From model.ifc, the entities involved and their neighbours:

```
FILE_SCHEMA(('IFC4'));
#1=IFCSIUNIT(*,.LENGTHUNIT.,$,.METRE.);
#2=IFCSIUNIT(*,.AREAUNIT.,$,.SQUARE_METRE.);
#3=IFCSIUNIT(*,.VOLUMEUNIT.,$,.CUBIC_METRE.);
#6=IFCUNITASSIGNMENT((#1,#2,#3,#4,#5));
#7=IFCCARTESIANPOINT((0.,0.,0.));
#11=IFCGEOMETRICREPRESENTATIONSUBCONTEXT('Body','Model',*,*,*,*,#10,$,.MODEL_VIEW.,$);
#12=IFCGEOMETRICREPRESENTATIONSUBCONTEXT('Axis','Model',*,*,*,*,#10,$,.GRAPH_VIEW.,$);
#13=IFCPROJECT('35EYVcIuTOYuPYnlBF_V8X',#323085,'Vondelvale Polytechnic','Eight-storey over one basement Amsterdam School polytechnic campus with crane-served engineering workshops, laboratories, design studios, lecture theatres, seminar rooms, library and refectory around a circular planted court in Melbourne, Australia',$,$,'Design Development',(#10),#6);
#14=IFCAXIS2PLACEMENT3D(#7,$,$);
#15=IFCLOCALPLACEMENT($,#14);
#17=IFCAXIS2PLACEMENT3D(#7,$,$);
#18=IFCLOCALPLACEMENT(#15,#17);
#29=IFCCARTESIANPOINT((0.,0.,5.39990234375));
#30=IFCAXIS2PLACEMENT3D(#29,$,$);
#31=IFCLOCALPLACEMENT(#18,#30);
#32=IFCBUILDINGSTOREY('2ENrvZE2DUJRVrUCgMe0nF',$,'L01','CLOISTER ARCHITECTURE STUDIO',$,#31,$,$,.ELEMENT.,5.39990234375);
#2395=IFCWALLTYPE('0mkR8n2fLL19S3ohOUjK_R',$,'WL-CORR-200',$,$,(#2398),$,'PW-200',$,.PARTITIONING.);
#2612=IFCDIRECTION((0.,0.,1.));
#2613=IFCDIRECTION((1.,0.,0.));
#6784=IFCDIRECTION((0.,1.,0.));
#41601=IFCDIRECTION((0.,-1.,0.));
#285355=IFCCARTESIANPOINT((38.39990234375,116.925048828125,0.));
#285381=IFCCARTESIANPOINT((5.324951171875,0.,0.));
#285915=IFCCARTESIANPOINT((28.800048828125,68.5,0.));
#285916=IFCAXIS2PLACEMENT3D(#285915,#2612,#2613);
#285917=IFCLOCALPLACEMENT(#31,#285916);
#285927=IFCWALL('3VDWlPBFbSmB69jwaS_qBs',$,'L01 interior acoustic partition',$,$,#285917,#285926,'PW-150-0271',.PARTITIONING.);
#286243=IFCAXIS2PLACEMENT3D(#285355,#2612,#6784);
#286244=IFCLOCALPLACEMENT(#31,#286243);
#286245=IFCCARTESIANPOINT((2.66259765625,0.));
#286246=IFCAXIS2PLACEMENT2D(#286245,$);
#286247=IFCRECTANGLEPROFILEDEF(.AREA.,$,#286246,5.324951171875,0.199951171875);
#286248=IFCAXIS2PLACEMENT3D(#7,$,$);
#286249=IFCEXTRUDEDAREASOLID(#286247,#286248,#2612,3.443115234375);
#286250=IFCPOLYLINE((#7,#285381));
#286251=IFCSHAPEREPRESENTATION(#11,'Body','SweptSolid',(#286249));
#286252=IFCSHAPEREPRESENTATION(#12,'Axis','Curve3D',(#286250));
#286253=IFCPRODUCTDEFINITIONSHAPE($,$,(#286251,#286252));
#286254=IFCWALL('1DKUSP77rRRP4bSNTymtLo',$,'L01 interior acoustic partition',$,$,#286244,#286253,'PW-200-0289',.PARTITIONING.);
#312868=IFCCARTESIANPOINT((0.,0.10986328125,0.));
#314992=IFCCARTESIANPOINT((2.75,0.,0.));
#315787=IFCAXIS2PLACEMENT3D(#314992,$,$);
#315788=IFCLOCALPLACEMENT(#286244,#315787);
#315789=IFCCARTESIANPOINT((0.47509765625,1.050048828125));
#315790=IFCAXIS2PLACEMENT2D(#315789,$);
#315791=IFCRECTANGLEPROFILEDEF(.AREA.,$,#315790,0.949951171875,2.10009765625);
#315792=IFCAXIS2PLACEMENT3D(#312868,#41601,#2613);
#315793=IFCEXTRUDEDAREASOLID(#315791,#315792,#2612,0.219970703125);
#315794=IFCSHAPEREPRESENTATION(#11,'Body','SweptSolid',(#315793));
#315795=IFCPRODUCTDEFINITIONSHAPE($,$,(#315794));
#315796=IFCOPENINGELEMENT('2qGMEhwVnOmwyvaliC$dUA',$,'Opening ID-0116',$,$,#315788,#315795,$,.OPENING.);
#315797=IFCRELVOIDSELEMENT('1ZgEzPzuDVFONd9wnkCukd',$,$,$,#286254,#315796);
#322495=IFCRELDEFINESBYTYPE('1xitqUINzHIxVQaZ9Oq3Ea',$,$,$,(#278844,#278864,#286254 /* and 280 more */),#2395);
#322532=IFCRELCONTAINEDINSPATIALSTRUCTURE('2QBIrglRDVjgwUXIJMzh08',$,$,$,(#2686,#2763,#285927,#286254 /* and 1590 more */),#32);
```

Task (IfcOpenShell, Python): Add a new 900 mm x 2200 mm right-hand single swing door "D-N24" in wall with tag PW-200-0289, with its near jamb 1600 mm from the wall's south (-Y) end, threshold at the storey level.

```python
import numpy as np
import ifcopenshell
import ifcopenshell.api.feature
import ifcopenshell.api.geometry
import ifcopenshell.api.root
import ifcopenshell.api.spatial
import ifcopenshell.geom
import ifcopenshell.util.element
import ifcopenshell.util.placement
import ifcopenshell.util.representation
import ifcopenshell.util.shape
import ifcopenshell.util.unit

model = ifcopenshell.open("model.ifc")
unit_scale = ifcopenshell.util.unit.calculate_unit_scale(model)
settings = ifcopenshell.geom.settings()


def volume(element):
    """Net volume in cubic metres, openings subtracted."""
    shape = ifcopenshell.geom.create_shape(settings, element)
    return ifcopenshell.util.shape.get_volume(shape.geometry)


wall = model.by_guid("1DKUSP77rRRP4bSNTymtLo")
storey = ifcopenshell.util.element.get_container(wall, ifc_class="IfcBuildingStorey")
context = ifcopenshell.util.representation.get_context(model, "Model", "Body", "MODEL_VIEW")
before = volume(wall)

width, height, from_end, sill = 0.9, 2.2, 1.6, 0.0  # metres

# The wall runs along its own X axis, and the end named is its -X end.
wall_shape = ifcopenshell.geom.create_shape(settings, wall)
x, y, z = ifcopenshell.util.shape.get_vertices(wall_shape.geometry).T
start = x.min() + from_end
face, thickness = float(y.min()), float(y.max() - y.min())
wall_matrix = ifcopenshell.util.placement.get_local_placement(wall.ObjectPlacement)
level = ifcopenshell.util.placement.get_local_placement(storey.ObjectPlacement)[2, 3]


def in_wall(x, y):
    """Placement at x, y metres in the wall's axes, at sill height."""
    matrix = wall_matrix.copy()
    matrix[:, 3] = wall_matrix @ np.array([x / unit_scale, y / unit_scale, 0.0, 1.0])
    matrix[2, 3] = level + sill / unit_scale
    return matrix


# Opening: a box that overshoots both wall faces by 50 mm.
opening = ifcopenshell.api.root.create_entity(model, ifc_class="IfcOpeningElement", predefined_type="OPENING")
box = ifcopenshell.api.geometry.add_wall_representation(
    model, context=context, length=width, height=height, thickness=thickness + 0.1
)
ifcopenshell.api.geometry.assign_representation(model, product=opening, representation=box)
ifcopenshell.api.geometry.edit_object_placement(model, product=opening, matrix=in_wall(start, face - 0.05), is_si=False)
ifcopenshell.api.feature.add_feature(model, feature=opening, element=wall)

door = ifcopenshell.api.root.create_entity(model, ifc_class="IfcDoor", name="D-N24", predefined_type="DOOR")
door.OverallWidth, door.OverallHeight = width / unit_scale, height / unit_scale
door.OperationType = "SINGLE_SWING_RIGHT"
body = ifcopenshell.api.geometry.add_door_representation(
    model,
    context=context,
    overall_width=door.OverallWidth,
    overall_height=door.OverallHeight,
    operation_type="SINGLE_SWING_RIGHT",
    lining_properties={"LiningDepth": thickness / unit_scale, "ThresholdDepth": thickness / unit_scale},
)
ifcopenshell.api.geometry.assign_representation(model, product=door, representation=body)
ifcopenshell.api.spatial.assign_container(model, products=[door], relating_structure=storey)
ifcopenshell.api.feature.add_filling(model, opening=opening, element=door)

# The lining spans the wall, so the door starts at the wall face.
ifcopenshell.api.geometry.edit_object_placement(model, product=door, matrix=in_wall(start, face), is_si=False)

after = volume(wall)

print(f"wall volume {before:.3f} -> {after:.3f} m3")

model.write("model_updated.ifc")
```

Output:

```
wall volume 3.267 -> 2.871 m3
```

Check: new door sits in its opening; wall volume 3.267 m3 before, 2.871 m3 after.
